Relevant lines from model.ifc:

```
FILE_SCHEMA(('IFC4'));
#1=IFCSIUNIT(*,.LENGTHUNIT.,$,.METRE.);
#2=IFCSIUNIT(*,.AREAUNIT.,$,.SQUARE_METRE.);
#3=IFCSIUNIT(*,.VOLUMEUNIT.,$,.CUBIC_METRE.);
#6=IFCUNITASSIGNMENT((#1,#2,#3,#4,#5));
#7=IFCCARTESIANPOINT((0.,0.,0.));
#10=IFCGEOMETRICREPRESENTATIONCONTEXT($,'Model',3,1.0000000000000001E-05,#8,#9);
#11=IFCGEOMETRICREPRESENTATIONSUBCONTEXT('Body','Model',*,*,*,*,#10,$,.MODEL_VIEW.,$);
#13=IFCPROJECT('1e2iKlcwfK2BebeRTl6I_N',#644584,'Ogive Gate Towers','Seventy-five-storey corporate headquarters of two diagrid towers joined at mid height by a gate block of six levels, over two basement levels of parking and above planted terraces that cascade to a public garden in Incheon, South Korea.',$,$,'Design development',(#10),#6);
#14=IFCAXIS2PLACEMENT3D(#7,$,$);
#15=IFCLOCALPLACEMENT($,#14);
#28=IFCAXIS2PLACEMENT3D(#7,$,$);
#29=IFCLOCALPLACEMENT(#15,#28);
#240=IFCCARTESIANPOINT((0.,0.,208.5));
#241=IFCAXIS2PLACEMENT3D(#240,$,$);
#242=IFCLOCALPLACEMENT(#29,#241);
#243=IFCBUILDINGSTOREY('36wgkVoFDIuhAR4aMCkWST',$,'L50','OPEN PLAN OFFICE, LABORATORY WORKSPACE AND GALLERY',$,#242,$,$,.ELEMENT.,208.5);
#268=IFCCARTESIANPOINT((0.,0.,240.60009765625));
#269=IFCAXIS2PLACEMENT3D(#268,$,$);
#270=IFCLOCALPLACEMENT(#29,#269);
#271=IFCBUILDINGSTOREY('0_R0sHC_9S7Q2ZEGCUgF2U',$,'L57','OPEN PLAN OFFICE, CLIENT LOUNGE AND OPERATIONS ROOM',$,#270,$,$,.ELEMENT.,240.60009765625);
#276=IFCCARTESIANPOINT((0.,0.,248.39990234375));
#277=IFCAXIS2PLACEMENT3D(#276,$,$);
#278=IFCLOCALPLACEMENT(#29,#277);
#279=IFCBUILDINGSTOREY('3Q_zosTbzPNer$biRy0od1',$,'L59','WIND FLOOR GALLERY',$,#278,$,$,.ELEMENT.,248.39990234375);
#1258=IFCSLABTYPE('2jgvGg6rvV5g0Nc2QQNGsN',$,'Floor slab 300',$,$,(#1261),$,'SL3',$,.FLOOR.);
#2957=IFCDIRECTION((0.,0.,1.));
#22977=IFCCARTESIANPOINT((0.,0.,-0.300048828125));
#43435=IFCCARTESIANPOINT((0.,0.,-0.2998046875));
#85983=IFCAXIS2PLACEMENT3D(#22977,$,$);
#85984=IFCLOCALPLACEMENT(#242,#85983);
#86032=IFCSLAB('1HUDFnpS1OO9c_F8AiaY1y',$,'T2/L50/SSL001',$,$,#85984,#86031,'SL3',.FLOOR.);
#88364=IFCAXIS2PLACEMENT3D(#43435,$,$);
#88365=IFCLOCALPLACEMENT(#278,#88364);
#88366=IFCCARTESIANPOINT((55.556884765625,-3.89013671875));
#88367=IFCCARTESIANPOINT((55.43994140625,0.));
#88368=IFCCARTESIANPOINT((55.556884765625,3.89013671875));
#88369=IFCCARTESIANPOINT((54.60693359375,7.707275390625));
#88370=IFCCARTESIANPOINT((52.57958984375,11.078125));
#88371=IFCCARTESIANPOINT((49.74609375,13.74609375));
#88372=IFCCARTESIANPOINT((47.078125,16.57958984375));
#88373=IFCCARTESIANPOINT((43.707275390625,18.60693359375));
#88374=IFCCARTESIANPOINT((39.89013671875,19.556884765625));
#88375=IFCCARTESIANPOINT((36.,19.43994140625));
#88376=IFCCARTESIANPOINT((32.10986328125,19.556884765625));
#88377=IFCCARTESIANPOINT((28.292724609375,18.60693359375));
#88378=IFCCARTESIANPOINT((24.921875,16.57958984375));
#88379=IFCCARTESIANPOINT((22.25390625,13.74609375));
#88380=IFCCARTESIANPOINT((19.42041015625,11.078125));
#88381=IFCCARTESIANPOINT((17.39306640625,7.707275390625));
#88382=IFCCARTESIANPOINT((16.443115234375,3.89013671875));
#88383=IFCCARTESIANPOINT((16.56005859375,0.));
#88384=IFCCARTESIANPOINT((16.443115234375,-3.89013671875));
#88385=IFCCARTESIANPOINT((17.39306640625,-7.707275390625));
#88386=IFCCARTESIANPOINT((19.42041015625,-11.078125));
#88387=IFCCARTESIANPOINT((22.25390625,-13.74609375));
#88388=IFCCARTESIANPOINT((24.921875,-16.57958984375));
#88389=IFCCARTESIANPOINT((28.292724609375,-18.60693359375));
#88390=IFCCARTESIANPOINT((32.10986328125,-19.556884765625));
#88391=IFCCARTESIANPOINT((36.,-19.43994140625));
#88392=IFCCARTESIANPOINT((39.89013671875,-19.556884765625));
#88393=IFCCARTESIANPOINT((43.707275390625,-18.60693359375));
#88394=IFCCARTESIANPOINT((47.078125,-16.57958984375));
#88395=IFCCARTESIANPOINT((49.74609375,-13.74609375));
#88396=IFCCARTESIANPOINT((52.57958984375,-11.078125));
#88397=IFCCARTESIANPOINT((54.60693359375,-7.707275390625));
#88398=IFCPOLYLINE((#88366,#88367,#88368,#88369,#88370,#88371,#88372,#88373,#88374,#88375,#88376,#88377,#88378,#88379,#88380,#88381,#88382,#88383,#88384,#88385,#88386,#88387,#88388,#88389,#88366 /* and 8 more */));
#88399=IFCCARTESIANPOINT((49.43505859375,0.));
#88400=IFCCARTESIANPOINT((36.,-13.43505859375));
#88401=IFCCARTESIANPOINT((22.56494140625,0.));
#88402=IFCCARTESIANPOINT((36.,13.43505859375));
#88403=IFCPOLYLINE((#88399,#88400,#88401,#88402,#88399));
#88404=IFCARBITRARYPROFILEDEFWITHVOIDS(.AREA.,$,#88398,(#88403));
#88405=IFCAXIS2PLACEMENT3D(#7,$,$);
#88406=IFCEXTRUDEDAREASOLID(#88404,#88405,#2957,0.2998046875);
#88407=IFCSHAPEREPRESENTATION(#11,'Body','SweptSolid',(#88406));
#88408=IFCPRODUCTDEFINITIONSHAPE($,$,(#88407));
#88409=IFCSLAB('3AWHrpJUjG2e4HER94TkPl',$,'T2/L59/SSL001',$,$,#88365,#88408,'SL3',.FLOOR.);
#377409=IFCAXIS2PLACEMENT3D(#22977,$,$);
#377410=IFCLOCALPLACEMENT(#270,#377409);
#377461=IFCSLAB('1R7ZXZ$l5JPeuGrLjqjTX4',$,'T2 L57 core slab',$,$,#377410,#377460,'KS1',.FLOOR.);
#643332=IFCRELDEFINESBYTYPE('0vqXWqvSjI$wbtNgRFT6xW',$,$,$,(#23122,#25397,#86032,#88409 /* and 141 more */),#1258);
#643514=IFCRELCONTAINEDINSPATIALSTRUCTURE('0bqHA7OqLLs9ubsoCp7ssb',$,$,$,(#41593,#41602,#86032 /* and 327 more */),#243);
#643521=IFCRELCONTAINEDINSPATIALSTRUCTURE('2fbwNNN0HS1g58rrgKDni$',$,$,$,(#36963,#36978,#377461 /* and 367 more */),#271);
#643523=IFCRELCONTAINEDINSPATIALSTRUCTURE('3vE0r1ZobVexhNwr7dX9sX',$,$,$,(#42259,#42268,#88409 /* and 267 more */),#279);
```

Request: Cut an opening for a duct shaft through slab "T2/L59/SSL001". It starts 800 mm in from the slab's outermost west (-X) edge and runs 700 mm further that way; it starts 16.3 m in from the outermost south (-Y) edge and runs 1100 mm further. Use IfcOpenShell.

```python
import numpy as np
import ifcopenshell
import ifcopenshell.api.feature
import ifcopenshell.api.geometry
import ifcopenshell.api.root
import ifcopenshell.geom
import ifcopenshell.util.placement
import ifcopenshell.util.representation
import ifcopenshell.util.shape
import ifcopenshell.util.unit

model = ifcopenshell.open("model.ifc")
unit_scale = ifcopenshell.util.unit.calculate_unit_scale(model)
settings = ifcopenshell.geom.settings()


def volume(element):
    """Net volume in cubic metres, openings subtracted."""
    shape = ifcopenshell.geom.create_shape(settings, element)
    return ifcopenshell.util.shape.get_volume(shape.geometry)


slab = model.by_id(88409)
before = volume(slab)

# Extent in the slab's own axes, in metres. The edges named are its -X and -Y sides.
slab_shape = ifcopenshell.geom.create_shape(settings, slab)
vertices = ifcopenshell.util.shape.get_vertices(slab_shape.geometry)
x_min, y_min, bottom = vertices.min(axis=0)
top = vertices[:, 2].max()

opening = ifcopenshell.api.root.create_entity(model, ifc_class="IfcOpeningElement", name="Duct shaft opening", predefined_type="OPENING")
context = ifcopenshell.util.representation.get_context(model, "Model", "Body", "MODEL_VIEW")
width, depth = 0.7, 1.1
outline = [(0.0, 0.0), (width, 0.0), (width, depth), (0.0, depth), (0.0, 0.0)]
# Overshoot both faces by 50 mm so the cut is clean.
shape = ifcopenshell.api.geometry.add_slab_representation(
    model, context=context, depth=top - bottom + 0.1, polyline=outline
)
ifcopenshell.api.geometry.assign_representation(model, product=opening, representation=shape)

matrix = ifcopenshell.util.placement.get_local_placement(slab.ObjectPlacement)
matrix[:, 3] = matrix @ np.append(np.array([x_min + 0.8, y_min + 16.3, bottom - 0.05]) / unit_scale, 1.0)
ifcopenshell.api.geometry.edit_object_placement(model, product=opening, matrix=matrix, is_si=False)
ifcopenshell.api.feature.add_feature(model, feature=opening, element=slab)

after = volume(slab)

print(f"slab volume {before:.3f} -> {after:.3f} m3")

model.write("model_rev.ifc")
```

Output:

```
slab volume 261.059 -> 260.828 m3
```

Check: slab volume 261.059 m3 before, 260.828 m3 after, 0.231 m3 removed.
